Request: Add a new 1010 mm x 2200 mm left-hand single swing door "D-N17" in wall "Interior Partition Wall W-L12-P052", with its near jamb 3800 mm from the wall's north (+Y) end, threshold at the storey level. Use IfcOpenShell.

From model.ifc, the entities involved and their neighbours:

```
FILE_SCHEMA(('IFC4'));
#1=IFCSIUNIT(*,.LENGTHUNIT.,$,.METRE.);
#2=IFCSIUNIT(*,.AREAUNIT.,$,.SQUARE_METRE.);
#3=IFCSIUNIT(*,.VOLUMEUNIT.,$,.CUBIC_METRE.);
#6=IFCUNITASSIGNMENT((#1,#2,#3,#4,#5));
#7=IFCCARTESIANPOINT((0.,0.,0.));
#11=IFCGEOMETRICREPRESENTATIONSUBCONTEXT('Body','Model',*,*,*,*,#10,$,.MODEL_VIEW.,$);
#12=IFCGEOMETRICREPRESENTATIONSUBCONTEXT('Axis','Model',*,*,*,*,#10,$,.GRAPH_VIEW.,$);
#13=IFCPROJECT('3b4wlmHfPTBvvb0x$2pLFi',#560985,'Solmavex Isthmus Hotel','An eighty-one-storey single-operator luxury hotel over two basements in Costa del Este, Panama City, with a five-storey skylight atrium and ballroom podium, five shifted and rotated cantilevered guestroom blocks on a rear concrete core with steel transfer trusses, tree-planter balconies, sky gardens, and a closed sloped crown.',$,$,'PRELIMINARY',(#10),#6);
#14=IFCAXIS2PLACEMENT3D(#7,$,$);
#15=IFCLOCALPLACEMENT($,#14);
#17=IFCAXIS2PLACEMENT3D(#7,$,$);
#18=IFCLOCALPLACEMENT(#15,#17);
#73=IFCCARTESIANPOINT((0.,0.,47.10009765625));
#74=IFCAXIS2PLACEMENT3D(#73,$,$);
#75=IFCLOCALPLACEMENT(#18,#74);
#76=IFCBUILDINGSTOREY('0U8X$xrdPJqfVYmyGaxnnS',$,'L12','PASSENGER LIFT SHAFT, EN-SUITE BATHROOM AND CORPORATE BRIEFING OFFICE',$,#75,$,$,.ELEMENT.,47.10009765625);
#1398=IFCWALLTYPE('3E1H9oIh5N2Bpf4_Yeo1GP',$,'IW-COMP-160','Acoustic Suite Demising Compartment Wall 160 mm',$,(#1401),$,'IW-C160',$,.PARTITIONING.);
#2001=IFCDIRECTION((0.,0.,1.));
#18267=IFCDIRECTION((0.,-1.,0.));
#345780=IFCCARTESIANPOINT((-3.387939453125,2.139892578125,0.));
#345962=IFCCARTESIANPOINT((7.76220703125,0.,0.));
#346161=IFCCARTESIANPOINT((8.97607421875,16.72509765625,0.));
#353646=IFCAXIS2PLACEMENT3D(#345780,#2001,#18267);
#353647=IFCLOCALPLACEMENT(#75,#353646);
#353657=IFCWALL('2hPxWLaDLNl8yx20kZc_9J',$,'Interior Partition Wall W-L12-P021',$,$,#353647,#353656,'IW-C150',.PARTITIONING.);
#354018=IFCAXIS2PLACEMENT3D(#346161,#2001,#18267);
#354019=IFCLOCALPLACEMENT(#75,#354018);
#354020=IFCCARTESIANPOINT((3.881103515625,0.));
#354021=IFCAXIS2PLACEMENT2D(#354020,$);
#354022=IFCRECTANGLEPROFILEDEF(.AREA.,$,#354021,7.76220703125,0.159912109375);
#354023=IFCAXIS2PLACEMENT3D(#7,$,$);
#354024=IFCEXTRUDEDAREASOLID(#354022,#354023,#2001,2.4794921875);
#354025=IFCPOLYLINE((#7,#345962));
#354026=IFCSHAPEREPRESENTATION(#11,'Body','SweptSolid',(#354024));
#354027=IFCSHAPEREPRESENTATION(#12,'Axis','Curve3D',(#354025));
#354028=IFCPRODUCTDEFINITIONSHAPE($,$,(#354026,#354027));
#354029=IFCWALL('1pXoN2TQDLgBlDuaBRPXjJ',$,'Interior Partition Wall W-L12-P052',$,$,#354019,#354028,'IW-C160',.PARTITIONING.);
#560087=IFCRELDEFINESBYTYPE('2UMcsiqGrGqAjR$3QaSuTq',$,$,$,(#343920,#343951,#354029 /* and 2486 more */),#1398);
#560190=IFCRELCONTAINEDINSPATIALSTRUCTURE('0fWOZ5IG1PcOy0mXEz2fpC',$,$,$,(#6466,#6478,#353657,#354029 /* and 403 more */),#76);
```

```python
import numpy as np
import ifcopenshell
import ifcopenshell.api.feature
import ifcopenshell.api.geometry
import ifcopenshell.api.root
import ifcopenshell.api.spatial
import ifcopenshell.geom
import ifcopenshell.util.element
import ifcopenshell.util.placement
import ifcopenshell.util.representation
import ifcopenshell.util.shape
import ifcopenshell.util.unit

model = ifcopenshell.open("model.ifc")
unit_scale = ifcopenshell.util.unit.calculate_unit_scale(model)
settings = ifcopenshell.geom.settings()


def volume(element):
    """Net volume in cubic metres, openings subtracted."""
    shape = ifcopenshell.geom.create_shape(settings, element)
    return ifcopenshell.util.shape.get_volume(shape.geometry)


wall = model.by_guid("1pXoN2TQDLgBlDuaBRPXjJ")
storey = ifcopenshell.util.element.get_container(wall, ifc_class="IfcBuildingStorey")
context = ifcopenshell.util.representation.get_context(model, "Model", "Body", "MODEL_VIEW")
before = volume(wall)

width, height, from_end, sill = 1.01, 2.2, 3.8, 0.0  # metres

# The wall runs along its own X axis, and the end named is its -X end.
wall_shape = ifcopenshell.geom.create_shape(settings, wall)
x, y, z = ifcopenshell.util.shape.get_vertices(wall_shape.geometry).T
start = x.min() + from_end
face, thickness = float(y.min()), float(y.max() - y.min())
wall_matrix = ifcopenshell.util.placement.get_local_placement(wall.ObjectPlacement)
level = ifcopenshell.util.placement.get_local_placement(storey.ObjectPlacement)[2, 3]


def in_wall(x, y):
    """Placement at x, y metres in the wall's axes, at sill height."""
    matrix = wall_matrix.copy()
    matrix[:, 3] = wall_matrix @ np.array([x / unit_scale, y / unit_scale, 0.0, 1.0])
    matrix[2, 3] = level + sill / unit_scale
    return matrix


# Opening: a box that overshoots both wall faces by 50 mm.
opening = ifcopenshell.api.root.create_entity(model, ifc_class="IfcOpeningElement", predefined_type="OPENING")
box = ifcopenshell.api.geometry.add_wall_representation(
    model, context=context, length=width, height=height, thickness=thickness + 0.1
)
ifcopenshell.api.geometry.assign_representation(model, product=opening, representation=box)
ifcopenshell.api.geometry.edit_object_placement(model, product=opening, matrix=in_wall(start, face - 0.05), is_si=False)
ifcopenshell.api.feature.add_feature(model, feature=opening, element=wall)

door = ifcopenshell.api.root.create_entity(model, ifc_class="IfcDoor", name="D-N17", predefined_type="DOOR")
door.OverallWidth, door.OverallHeight = width / unit_scale, height / unit_scale
door.OperationType = "SINGLE_SWING_LEFT"
body = ifcopenshell.api.geometry.add_door_representation(
    model,
    context=context,
    overall_width=door.OverallWidth,
    overall_height=door.OverallHeight,
    operation_type="SINGLE_SWING_LEFT",
    lining_properties={"LiningDepth": thickness / unit_scale, "ThresholdDepth": thickness / unit_scale},
)
ifcopenshell.api.geometry.assign_representation(model, product=door, representation=body)
ifcopenshell.api.spatial.assign_container(model, products=[door], relating_structure=storey)
ifcopenshell.api.feature.add_filling(model, opening=opening, element=door)

# The lining spans the wall, so the door starts at the wall face.
ifcopenshell.api.geometry.edit_object_placement(model, product=door, matrix=in_wall(start, face), is_si=False)

after = volume(wall)

print(f"wall volume {before:.3f} -> {after:.3f} m3")

model.write("model-out.ifc")
```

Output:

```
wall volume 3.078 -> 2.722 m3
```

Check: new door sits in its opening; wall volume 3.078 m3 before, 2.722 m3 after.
